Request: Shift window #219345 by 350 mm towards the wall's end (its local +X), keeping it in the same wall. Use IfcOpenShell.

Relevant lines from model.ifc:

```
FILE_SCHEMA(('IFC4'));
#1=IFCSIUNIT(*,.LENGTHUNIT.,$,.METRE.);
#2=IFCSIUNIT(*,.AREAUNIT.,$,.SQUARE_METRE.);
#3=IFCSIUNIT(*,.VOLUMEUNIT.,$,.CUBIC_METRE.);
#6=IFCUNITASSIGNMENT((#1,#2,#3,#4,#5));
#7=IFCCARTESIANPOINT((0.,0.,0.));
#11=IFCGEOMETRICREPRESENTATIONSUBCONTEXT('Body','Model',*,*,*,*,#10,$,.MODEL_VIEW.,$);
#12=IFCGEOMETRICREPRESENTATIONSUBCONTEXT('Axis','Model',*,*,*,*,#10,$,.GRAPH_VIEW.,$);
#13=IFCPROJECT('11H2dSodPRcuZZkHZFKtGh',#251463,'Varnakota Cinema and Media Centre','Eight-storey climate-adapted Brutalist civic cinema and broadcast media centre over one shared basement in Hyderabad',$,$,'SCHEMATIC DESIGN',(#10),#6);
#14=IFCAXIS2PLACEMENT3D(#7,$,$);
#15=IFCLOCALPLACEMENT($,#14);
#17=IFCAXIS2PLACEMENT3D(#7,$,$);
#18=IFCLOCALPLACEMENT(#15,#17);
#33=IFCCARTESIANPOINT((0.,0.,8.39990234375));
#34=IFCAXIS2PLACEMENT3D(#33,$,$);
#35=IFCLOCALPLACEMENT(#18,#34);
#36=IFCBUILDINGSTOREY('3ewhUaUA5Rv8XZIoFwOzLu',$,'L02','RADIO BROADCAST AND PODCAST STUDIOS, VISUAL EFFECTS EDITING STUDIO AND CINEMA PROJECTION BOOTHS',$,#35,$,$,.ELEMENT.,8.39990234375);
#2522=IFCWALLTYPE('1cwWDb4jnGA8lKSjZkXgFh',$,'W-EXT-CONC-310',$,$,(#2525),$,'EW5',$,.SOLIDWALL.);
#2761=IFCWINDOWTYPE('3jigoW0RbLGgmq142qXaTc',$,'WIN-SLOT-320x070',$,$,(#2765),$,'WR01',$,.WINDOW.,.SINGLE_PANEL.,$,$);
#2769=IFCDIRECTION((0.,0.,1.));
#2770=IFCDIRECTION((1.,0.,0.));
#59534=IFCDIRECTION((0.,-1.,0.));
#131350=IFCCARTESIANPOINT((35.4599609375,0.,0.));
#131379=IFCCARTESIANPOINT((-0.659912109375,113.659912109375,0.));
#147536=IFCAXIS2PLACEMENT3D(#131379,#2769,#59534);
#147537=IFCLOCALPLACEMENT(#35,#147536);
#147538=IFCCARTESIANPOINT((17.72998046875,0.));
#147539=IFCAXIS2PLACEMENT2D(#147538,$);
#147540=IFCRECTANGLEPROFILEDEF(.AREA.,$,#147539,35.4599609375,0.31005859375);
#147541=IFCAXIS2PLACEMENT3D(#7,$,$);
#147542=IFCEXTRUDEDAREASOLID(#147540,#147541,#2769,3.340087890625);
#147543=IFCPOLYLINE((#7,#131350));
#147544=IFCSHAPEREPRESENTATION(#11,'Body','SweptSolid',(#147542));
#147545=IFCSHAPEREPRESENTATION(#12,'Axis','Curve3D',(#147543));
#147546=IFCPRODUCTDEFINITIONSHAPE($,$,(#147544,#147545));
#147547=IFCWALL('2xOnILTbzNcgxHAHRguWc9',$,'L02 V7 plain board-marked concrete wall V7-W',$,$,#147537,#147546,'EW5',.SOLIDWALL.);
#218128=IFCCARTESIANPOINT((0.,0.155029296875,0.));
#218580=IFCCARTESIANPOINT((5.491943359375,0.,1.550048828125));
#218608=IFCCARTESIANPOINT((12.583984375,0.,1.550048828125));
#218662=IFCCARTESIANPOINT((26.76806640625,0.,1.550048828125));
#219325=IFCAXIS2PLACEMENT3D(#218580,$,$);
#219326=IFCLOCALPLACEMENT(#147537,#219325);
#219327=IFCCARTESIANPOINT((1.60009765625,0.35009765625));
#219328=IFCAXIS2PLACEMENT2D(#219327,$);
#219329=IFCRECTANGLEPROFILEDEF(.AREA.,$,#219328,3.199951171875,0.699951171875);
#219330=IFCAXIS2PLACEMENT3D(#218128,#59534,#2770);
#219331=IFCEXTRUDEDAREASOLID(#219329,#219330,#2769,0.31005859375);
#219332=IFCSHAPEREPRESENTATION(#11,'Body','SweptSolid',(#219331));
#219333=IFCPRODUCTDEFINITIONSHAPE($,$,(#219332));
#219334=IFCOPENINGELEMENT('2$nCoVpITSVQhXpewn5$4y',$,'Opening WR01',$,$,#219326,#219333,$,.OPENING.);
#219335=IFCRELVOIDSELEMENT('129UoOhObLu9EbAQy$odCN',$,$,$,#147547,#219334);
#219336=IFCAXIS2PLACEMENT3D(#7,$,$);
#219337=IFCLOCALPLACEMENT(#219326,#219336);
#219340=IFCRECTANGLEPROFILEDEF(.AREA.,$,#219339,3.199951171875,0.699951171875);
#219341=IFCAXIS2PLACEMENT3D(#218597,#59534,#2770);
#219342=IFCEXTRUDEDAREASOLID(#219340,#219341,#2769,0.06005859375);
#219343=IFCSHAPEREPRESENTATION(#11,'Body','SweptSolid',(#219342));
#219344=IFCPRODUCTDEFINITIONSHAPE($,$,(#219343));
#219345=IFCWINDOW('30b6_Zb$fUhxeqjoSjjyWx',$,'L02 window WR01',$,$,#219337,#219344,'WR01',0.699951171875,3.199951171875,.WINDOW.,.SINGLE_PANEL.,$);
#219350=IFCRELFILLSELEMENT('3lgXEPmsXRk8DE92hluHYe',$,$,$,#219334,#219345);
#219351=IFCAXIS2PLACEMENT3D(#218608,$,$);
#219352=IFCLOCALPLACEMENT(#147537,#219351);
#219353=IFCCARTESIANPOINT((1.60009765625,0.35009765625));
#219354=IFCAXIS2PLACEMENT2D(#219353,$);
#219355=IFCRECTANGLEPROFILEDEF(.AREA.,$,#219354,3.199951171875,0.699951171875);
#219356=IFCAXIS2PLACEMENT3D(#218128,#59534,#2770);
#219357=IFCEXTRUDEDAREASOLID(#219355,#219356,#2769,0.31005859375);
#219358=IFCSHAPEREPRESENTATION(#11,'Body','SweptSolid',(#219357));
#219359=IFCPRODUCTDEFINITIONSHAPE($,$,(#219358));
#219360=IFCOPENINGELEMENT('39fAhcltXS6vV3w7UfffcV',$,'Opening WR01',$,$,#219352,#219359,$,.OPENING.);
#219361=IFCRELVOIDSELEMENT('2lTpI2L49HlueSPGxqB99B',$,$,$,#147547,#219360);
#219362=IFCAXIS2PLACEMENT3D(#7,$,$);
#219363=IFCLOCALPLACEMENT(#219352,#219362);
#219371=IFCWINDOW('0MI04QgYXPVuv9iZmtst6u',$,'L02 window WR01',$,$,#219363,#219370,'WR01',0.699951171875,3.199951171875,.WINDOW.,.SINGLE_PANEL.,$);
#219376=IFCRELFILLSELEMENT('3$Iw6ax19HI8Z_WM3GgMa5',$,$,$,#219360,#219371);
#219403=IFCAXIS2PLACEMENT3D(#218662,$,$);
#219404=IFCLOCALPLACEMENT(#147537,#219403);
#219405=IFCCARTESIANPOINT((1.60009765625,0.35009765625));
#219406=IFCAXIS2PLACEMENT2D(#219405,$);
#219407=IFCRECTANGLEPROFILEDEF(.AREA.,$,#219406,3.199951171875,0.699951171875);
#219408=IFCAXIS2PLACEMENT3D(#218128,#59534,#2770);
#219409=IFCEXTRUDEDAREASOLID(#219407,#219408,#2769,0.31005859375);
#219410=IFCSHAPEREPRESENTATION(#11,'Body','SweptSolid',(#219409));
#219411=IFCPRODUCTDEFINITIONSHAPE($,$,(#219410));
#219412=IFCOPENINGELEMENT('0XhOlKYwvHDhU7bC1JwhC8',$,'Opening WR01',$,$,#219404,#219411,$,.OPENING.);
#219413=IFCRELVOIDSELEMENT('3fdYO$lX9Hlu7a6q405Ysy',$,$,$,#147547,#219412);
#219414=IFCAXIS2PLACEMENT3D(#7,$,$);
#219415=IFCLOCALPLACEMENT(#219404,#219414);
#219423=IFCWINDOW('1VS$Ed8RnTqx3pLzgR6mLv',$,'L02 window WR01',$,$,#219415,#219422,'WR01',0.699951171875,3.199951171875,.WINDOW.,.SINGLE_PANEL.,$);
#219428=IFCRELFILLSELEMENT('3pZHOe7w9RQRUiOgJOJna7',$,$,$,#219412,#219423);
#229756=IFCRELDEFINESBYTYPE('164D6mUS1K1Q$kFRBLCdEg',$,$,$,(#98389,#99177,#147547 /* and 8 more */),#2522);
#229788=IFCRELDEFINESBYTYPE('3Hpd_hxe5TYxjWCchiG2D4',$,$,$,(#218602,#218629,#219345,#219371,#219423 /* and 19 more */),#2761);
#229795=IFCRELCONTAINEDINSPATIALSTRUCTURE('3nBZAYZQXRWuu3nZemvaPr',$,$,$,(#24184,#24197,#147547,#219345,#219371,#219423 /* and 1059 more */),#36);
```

```python
import ifcopenshell
import ifcopenshell.api.geometry
import ifcopenshell.util.placement

model = ifcopenshell.open("model.ifc")

window = model.by_id(219345)
opening = window.FillsVoids[0].RelatingOpeningElement
wall = opening.VoidsElements[0].RelatingBuildingElement

wall_matrix = ifcopenshell.util.placement.get_local_placement(wall.ObjectPlacement)
shift = wall_matrix[:3, 0] * 0.35
before = ifcopenshell.util.placement.get_local_placement(window.ObjectPlacement)[:3, 3].copy()

# The window is placed relative to its opening, so it follows when the opening moves.
matrix = ifcopenshell.util.placement.get_local_placement(opening.ObjectPlacement)
matrix[:3, 3] += shift
ifcopenshell.api.geometry.edit_object_placement(
    model, product=opening, matrix=matrix, is_si=False, should_transform_children=True
)

after = ifcopenshell.util.placement.get_local_placement(window.ObjectPlacement)[:3, 3]
print("window moved by", (after - before).round(3) + 0.0)

model.write("model_rev.ifc")
```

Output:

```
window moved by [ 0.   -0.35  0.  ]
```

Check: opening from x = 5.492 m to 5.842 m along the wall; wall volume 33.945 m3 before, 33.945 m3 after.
